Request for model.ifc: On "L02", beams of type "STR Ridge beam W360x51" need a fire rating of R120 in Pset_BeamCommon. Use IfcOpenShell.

First a look at what the model holds.

```python
import ifcopenshell
import ifcopenshell.util.element

model = ifcopenshell.open("model.ifc")
print(model.schema)
storey = next(s for s in model.by_type("IfcBuildingStorey") if s.Name == "L02")
beams = [e for e in ifcopenshell.util.element.get_decomposition(storey) if e.is_a("IfcBeam")]
seen = {}
for e in beams:
    element_type = ifcopenshell.util.element.get_type(e)
    key = (element_type.Name if element_type != e and element_type else None, ifcopenshell.util.element.get_pset(e, "Pset_BeamCommon", "FireRating"))
    seen[key] = seen.get(key, 0) + 1
for (name, value), count in sorted(seen.items(), key=str):
    print(count, "x", name, "|", value)
```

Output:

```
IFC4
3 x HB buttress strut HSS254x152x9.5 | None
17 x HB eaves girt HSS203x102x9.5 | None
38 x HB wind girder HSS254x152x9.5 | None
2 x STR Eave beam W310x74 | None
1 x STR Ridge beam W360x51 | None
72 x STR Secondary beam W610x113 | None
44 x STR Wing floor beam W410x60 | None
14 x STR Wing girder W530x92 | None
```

```python
import ifcopenshell
import ifcopenshell.api.pset
import ifcopenshell.util.element

model = ifcopenshell.open("model.ifc")

storey = next(s for s in model.by_type("IfcBuildingStorey") if s.Name == "L02")
beams = [e for e in ifcopenshell.util.element.get_decomposition(storey) if e.is_a("IfcBeam")]

count = 0
for e in beams:
    element_type = ifcopenshell.util.element.get_type(e)
    if element_type in (None, e) or element_type.Name != "STR Ridge beam W360x51":
        continue
    # add_pset returns the element's existing set when there is one.
    pset = ifcopenshell.api.pset.add_pset(model, product=e, name="Pset_BeamCommon")
    ifcopenshell.api.pset.edit_pset(model, pset=pset, properties={"FireRating": "R120"})
    count += 1

print(count, "beams updated")

model.write("model_rev.ifc")
```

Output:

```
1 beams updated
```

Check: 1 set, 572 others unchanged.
